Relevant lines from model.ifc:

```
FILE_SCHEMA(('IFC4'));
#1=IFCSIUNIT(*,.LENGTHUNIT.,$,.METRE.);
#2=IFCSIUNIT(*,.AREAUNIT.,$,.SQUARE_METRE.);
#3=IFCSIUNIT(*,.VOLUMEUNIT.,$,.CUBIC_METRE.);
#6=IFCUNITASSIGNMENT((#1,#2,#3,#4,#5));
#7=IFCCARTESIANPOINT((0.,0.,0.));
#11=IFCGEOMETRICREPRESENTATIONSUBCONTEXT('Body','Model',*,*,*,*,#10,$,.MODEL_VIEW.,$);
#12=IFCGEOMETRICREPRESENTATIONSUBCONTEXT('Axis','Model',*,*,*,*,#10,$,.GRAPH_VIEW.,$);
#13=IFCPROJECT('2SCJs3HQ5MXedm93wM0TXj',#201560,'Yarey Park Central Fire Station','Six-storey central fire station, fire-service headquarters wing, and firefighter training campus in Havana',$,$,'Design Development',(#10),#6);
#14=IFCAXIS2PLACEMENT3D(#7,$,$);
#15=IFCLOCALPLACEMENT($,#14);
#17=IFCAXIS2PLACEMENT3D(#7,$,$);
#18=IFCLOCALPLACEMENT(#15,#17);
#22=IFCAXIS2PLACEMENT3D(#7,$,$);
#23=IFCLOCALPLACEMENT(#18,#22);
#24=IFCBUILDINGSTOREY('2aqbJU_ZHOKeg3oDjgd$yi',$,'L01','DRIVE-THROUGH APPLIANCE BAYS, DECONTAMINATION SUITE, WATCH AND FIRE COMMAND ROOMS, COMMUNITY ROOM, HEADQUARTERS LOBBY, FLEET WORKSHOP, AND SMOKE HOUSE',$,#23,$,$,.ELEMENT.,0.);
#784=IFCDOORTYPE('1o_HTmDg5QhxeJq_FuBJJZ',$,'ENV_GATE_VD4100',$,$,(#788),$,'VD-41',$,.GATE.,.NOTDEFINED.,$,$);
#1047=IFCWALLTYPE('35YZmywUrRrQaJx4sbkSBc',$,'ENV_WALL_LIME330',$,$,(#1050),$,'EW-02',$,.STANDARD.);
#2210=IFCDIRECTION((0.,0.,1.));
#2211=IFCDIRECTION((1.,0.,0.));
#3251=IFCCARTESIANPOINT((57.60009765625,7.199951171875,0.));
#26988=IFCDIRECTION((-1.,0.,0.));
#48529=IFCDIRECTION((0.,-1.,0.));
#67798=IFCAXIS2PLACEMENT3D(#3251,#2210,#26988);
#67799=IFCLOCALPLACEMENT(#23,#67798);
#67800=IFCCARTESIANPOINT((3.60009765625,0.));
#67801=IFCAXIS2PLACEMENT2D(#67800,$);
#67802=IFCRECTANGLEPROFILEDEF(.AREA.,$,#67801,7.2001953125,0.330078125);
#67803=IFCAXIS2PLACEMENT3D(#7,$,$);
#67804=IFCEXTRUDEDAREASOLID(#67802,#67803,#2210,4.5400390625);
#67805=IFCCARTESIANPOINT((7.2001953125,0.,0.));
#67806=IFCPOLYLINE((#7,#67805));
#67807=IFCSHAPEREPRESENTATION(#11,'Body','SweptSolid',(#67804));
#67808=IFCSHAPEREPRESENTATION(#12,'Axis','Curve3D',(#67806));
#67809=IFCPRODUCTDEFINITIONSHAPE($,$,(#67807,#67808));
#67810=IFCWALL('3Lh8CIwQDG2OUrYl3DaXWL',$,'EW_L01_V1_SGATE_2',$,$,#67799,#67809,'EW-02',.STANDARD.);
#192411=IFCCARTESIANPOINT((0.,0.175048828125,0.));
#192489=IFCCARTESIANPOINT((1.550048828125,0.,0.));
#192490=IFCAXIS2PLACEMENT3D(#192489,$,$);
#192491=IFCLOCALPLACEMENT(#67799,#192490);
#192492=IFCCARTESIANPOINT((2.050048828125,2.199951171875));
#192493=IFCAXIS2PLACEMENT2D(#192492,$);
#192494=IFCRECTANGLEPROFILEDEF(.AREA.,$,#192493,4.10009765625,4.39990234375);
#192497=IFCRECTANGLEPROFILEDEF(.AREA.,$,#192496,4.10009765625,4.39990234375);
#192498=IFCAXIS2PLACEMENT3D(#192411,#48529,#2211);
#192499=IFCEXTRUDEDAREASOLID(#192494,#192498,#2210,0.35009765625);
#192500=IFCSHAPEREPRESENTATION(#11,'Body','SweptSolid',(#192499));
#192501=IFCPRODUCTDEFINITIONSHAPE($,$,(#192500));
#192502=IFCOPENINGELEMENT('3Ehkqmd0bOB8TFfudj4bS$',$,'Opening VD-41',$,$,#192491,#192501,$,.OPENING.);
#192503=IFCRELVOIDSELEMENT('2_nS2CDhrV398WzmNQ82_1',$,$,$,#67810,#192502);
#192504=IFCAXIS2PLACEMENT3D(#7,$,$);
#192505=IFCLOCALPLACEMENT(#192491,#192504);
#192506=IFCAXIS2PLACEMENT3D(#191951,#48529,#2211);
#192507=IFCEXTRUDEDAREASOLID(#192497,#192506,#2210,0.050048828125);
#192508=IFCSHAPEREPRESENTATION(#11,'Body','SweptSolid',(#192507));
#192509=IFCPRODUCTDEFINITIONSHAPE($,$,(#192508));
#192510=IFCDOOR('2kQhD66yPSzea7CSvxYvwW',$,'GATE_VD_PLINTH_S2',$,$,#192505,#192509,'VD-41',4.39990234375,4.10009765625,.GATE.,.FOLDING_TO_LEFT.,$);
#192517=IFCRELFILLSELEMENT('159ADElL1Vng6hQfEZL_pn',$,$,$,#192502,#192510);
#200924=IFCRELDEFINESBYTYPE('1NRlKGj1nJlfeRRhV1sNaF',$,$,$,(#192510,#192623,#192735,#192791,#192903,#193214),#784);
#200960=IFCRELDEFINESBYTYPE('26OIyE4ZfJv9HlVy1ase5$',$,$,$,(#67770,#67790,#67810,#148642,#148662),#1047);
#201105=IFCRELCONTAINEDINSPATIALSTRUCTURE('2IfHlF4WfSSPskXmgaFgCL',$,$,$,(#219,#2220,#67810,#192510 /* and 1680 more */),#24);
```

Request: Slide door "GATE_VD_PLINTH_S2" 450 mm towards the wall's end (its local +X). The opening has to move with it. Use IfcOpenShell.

```python
import ifcopenshell
import ifcopenshell.api.geometry
import ifcopenshell.util.placement

model = ifcopenshell.open("model.ifc")

door = model.by_id(192510)
opening = door.FillsVoids[0].RelatingOpeningElement
wall = opening.VoidsElements[0].RelatingBuildingElement

wall_matrix = ifcopenshell.util.placement.get_local_placement(wall.ObjectPlacement)
shift = wall_matrix[:3, 0] * 0.45
before = ifcopenshell.util.placement.get_local_placement(door.ObjectPlacement)[:3, 3].copy()

# The door is placed relative to its opening, so it follows when the opening moves.
matrix = ifcopenshell.util.placement.get_local_placement(opening.ObjectPlacement)
matrix[:3, 3] += shift
ifcopenshell.api.geometry.edit_object_placement(
    model, product=opening, matrix=matrix, is_si=False, should_transform_children=True
)

after = ifcopenshell.util.placement.get_local_placement(door.ObjectPlacement)[:3, 3]
print("door moved by", (after - before).round(3) + 0.0)

model.write("model-out.ifc")
```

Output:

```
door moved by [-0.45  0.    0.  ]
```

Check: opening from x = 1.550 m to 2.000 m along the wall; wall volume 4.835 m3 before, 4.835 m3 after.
